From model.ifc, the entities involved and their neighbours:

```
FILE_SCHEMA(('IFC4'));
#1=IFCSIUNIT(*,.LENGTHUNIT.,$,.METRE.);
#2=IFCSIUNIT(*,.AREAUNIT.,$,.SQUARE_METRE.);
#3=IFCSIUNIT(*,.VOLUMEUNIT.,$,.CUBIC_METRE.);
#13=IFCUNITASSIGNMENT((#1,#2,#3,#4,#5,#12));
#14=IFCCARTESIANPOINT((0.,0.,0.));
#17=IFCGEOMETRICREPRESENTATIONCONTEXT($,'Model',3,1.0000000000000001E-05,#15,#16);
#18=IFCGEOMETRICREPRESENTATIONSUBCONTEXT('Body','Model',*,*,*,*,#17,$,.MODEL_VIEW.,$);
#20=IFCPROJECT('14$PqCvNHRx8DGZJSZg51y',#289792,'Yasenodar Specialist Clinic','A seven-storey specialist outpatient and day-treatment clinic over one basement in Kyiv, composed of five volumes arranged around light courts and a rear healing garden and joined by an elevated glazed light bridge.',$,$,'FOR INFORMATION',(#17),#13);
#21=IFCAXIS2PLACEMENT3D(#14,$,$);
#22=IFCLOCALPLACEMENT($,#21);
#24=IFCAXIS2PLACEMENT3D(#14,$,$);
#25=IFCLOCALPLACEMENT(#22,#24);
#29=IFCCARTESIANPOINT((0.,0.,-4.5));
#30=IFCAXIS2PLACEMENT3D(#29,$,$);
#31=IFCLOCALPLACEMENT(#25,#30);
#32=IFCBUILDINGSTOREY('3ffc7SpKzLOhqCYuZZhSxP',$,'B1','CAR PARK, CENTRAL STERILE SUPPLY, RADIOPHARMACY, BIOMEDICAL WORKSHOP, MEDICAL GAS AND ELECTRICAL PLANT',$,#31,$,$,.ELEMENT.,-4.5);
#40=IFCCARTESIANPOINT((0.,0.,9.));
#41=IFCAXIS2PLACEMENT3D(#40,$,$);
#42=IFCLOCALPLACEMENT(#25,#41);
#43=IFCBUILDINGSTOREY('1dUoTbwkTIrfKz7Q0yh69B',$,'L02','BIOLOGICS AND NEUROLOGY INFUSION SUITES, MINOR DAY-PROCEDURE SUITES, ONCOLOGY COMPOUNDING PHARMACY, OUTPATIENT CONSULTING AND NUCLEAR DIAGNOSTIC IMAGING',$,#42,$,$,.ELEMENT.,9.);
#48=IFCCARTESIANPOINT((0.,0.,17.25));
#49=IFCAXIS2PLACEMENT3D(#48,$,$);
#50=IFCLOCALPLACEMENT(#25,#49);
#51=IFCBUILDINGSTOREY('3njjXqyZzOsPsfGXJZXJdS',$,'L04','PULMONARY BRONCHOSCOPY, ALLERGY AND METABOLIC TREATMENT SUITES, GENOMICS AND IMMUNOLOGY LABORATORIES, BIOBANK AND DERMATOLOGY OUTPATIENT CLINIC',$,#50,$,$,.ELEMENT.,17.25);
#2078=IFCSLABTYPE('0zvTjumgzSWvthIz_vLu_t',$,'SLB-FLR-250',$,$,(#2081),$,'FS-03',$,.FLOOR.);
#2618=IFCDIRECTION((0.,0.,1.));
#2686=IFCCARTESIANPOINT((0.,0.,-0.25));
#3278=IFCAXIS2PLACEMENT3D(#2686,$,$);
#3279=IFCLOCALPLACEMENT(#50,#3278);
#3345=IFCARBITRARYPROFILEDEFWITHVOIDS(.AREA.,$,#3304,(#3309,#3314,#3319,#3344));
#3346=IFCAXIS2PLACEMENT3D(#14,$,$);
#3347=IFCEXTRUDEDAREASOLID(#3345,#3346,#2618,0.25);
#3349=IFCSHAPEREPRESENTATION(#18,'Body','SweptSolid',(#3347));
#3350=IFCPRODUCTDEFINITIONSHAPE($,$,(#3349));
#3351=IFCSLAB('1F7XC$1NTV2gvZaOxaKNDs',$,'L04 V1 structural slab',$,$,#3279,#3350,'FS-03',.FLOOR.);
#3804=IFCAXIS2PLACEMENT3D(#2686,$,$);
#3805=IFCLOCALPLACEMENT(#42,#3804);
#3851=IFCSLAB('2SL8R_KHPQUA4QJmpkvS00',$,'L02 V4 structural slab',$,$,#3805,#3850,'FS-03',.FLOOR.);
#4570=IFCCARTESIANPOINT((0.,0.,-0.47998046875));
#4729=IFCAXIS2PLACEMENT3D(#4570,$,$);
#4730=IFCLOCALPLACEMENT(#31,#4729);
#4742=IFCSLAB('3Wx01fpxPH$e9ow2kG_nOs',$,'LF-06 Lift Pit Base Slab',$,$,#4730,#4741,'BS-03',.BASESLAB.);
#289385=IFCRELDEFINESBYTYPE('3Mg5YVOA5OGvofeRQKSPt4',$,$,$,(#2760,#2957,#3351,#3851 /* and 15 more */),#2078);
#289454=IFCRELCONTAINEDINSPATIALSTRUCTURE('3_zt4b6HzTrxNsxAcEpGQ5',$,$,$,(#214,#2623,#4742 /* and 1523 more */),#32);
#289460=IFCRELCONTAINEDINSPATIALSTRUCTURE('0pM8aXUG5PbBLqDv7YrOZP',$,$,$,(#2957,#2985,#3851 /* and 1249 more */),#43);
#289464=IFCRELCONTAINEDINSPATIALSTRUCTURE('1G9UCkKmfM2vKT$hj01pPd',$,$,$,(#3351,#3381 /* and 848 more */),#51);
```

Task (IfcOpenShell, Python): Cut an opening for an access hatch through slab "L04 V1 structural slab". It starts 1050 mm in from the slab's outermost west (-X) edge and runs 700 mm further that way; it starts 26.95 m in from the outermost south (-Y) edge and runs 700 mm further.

```python
import numpy as np
import ifcopenshell
import ifcopenshell.api.feature
import ifcopenshell.api.geometry
import ifcopenshell.api.root
import ifcopenshell.geom
import ifcopenshell.util.placement
import ifcopenshell.util.representation
import ifcopenshell.util.shape
import ifcopenshell.util.unit

model = ifcopenshell.open("model.ifc")
unit_scale = ifcopenshell.util.unit.calculate_unit_scale(model)
settings = ifcopenshell.geom.settings()


def volume(element):
    """Net volume in cubic metres, openings subtracted."""
    shape = ifcopenshell.geom.create_shape(settings, element)
    return ifcopenshell.util.shape.get_volume(shape.geometry)


slab = model.by_guid("1F7XC$1NTV2gvZaOxaKNDs")
before = volume(slab)

# Extent in the slab's own axes, in metres. The edges named are its -X and -Y sides.
slab_shape = ifcopenshell.geom.create_shape(settings, slab)
vertices = ifcopenshell.util.shape.get_vertices(slab_shape.geometry)
x_min, y_min, bottom = vertices.min(axis=0)
top = vertices[:, 2].max()

opening = ifcopenshell.api.root.create_entity(model, ifc_class="IfcOpeningElement", name="Access hatch opening", predefined_type="OPENING")
context = ifcopenshell.util.representation.get_context(model, "Model", "Body", "MODEL_VIEW")
width, depth = 0.7, 0.7
outline = [(0.0, 0.0), (width, 0.0), (width, depth), (0.0, depth), (0.0, 0.0)]
# Overshoot both faces by 50 mm so the cut is clean.
shape = ifcopenshell.api.geometry.add_slab_representation(
    model, context=context, depth=top - bottom + 0.1, polyline=outline
)
ifcopenshell.api.geometry.assign_representation(model, product=opening, representation=shape)

matrix = ifcopenshell.util.placement.get_local_placement(slab.ObjectPlacement)
matrix[:, 3] = matrix @ np.append(np.array([x_min + 1.05, y_min + 26.95, bottom - 0.05]) / unit_scale, 1.0)
ifcopenshell.api.geometry.edit_object_placement(model, product=opening, matrix=matrix, is_si=False)
ifcopenshell.api.feature.add_feature(model, feature=opening, element=slab)

after = volume(slab)

print(f"slab volume {before:.3f} -> {after:.3f} m3")

model.write("model-out.ifc")
```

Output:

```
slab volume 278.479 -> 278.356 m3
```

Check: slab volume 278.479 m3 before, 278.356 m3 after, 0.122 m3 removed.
